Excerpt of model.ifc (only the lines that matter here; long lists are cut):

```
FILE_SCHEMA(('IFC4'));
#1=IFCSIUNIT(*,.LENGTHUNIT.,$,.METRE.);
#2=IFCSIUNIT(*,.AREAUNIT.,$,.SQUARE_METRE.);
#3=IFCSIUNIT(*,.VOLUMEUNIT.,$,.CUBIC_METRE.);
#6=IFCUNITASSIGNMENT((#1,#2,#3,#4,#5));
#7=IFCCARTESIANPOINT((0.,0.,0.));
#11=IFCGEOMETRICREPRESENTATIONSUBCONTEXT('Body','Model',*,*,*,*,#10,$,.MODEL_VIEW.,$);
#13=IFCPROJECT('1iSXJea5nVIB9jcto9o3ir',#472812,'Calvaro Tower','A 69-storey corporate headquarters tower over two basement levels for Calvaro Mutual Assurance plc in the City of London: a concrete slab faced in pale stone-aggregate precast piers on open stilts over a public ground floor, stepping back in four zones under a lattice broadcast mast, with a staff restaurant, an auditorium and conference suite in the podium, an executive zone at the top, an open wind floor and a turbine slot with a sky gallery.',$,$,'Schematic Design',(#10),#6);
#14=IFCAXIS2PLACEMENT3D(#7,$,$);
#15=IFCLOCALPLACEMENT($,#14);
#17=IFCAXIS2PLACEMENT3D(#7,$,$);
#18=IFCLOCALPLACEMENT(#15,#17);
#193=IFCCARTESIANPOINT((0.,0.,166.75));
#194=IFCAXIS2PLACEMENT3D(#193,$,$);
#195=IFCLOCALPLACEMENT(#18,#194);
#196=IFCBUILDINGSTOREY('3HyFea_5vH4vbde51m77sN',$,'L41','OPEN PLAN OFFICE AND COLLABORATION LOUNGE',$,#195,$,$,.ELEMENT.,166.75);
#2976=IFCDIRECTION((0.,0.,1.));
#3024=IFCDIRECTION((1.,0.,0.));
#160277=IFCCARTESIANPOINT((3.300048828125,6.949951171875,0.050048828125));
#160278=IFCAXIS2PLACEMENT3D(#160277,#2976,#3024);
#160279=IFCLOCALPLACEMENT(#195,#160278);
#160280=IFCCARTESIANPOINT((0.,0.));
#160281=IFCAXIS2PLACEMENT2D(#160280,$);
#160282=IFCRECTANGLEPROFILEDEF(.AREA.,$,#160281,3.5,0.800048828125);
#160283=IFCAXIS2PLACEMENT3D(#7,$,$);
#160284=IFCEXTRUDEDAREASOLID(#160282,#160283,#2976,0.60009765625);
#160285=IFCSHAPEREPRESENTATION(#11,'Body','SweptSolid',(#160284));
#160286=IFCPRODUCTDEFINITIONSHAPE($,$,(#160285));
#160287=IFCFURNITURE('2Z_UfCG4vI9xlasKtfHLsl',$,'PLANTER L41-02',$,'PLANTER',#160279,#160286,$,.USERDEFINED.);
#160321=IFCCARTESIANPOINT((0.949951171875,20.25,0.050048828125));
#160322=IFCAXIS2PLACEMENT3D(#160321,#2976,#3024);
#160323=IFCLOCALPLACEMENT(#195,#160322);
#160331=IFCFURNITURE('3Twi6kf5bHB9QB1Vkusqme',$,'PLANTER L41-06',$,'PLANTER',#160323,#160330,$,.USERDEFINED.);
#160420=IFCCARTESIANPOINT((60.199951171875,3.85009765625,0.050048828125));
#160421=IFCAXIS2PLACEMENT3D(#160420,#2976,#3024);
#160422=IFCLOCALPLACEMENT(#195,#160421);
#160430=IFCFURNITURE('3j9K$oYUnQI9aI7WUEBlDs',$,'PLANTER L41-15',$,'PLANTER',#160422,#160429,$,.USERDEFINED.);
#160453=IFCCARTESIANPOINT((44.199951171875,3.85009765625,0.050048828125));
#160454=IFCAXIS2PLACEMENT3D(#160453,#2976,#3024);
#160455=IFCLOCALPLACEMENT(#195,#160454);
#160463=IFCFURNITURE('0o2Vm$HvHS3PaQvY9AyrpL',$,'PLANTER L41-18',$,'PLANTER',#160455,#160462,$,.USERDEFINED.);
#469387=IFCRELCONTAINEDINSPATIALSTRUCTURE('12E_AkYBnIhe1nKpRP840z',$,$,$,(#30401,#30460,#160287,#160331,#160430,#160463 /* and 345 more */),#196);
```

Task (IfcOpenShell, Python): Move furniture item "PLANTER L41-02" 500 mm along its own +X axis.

```python
import ifcopenshell
import ifcopenshell.api.geometry
import ifcopenshell.util.placement

model = ifcopenshell.open("model.ifc")

item = model.by_guid("2Z_UfCG4vI9xlasKtfHLsl")
matrix = ifcopenshell.util.placement.get_local_placement(item.ObjectPlacement)
matrix[:3, 3] += matrix[:3, 0] * 0.5
ifcopenshell.api.geometry.edit_object_placement(model, product=item, matrix=matrix, is_si=False)

print(ifcopenshell.util.placement.get_local_placement(item.ObjectPlacement).round(3) + 0.0)

model.write("model_updated.ifc")
```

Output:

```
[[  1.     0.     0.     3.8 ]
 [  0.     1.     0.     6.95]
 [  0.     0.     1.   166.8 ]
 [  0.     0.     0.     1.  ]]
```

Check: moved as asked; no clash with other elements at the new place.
